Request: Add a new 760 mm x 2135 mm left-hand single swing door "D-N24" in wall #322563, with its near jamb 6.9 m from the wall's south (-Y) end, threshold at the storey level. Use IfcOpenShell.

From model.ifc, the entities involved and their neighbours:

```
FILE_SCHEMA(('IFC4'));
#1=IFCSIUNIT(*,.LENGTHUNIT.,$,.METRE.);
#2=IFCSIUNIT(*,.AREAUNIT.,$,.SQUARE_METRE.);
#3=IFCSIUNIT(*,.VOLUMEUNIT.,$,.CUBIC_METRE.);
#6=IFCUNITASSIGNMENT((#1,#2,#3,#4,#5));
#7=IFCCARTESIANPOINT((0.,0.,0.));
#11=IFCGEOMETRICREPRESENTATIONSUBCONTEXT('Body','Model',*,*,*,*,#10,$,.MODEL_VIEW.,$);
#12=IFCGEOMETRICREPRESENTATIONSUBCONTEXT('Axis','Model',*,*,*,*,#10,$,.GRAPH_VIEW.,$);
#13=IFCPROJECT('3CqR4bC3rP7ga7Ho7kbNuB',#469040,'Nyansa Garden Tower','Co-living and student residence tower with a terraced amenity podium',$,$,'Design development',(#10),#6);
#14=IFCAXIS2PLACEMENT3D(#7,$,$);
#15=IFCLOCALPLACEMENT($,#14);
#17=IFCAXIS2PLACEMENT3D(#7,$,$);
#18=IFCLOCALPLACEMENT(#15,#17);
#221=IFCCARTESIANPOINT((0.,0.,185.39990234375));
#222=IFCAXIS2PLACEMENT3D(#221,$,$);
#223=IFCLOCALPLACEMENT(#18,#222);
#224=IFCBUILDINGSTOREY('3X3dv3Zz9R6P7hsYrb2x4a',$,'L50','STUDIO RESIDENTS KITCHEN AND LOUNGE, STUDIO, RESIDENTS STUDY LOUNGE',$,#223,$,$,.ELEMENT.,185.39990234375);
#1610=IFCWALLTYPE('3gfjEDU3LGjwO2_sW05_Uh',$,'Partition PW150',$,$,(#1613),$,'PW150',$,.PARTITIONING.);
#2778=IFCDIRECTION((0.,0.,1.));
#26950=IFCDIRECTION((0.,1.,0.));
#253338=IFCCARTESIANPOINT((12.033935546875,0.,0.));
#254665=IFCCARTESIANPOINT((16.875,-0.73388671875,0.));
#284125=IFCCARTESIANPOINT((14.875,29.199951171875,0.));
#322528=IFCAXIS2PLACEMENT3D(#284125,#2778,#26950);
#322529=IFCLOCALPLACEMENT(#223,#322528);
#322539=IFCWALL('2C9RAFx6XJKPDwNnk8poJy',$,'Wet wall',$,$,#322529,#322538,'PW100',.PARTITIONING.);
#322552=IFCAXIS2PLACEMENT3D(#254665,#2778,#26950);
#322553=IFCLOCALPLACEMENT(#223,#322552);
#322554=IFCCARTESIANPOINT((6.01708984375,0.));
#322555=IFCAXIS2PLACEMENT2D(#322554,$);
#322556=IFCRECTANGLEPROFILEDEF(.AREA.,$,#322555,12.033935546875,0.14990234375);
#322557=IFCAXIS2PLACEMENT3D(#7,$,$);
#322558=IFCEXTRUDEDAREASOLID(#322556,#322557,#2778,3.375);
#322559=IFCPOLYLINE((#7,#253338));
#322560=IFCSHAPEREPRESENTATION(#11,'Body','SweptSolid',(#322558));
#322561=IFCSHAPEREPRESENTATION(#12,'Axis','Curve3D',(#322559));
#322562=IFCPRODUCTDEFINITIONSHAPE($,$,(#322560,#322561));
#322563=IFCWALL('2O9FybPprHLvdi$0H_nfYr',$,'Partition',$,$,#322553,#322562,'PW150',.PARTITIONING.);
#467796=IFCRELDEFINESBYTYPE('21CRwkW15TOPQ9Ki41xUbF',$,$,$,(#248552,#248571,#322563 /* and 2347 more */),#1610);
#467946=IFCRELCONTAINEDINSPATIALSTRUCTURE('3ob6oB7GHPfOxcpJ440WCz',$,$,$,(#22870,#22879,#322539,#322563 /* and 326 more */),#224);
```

```python
import numpy as np
import ifcopenshell
import ifcopenshell.api.feature
import ifcopenshell.api.geometry
import ifcopenshell.api.root
import ifcopenshell.api.spatial
import ifcopenshell.geom
import ifcopenshell.util.element
import ifcopenshell.util.placement
import ifcopenshell.util.representation
import ifcopenshell.util.shape
import ifcopenshell.util.unit

model = ifcopenshell.open("model.ifc")
unit_scale = ifcopenshell.util.unit.calculate_unit_scale(model)
settings = ifcopenshell.geom.settings()


def volume(element):
    """Net volume in cubic metres, openings subtracted."""
    shape = ifcopenshell.geom.create_shape(settings, element)
    return ifcopenshell.util.shape.get_volume(shape.geometry)


wall = model.by_id(322563)
storey = ifcopenshell.util.element.get_container(wall, ifc_class="IfcBuildingStorey")
context = ifcopenshell.util.representation.get_context(model, "Model", "Body", "MODEL_VIEW")
before = volume(wall)

width, height, from_end, sill = 0.76, 2.135, 6.9, 0.0  # metres

# The wall runs along its own X axis, and the end named is its -X end.
wall_shape = ifcopenshell.geom.create_shape(settings, wall)
x, y, z = ifcopenshell.util.shape.get_vertices(wall_shape.geometry).T
start = x.min() + from_end
face, thickness = float(y.min()), float(y.max() - y.min())
wall_matrix = ifcopenshell.util.placement.get_local_placement(wall.ObjectPlacement)
level = ifcopenshell.util.placement.get_local_placement(storey.ObjectPlacement)[2, 3]


def in_wall(x, y):
    """Placement at x, y metres in the wall's axes, at sill height."""
    matrix = wall_matrix.copy()
    matrix[:, 3] = wall_matrix @ np.array([x / unit_scale, y / unit_scale, 0.0, 1.0])
    matrix[2, 3] = level + sill / unit_scale
    return matrix


# Opening: a box that overshoots both wall faces by 50 mm.
opening = ifcopenshell.api.root.create_entity(model, ifc_class="IfcOpeningElement", predefined_type="OPENING")
box = ifcopenshell.api.geometry.add_wall_representation(
    model, context=context, length=width, height=height, thickness=thickness + 0.1
)
ifcopenshell.api.geometry.assign_representation(model, product=opening, representation=box)
ifcopenshell.api.geometry.edit_object_placement(model, product=opening, matrix=in_wall(start, face - 0.05), is_si=False)
ifcopenshell.api.feature.add_feature(model, feature=opening, element=wall)

door = ifcopenshell.api.root.create_entity(model, ifc_class="IfcDoor", name="D-N24", predefined_type="DOOR")
door.OverallWidth, door.OverallHeight = width / unit_scale, height / unit_scale
door.OperationType = "SINGLE_SWING_LEFT"
body = ifcopenshell.api.geometry.add_door_representation(
    model,
    context=context,
    overall_width=door.OverallWidth,
    overall_height=door.OverallHeight,
    operation_type="SINGLE_SWING_LEFT",
    lining_properties={"LiningDepth": thickness / unit_scale, "ThresholdDepth": thickness / unit_scale},
)
ifcopenshell.api.geometry.assign_representation(model, product=door, representation=body)
ifcopenshell.api.spatial.assign_container(model, products=[door], relating_structure=storey)
ifcopenshell.api.feature.add_filling(model, opening=opening, element=door)

# The lining spans the wall, so the door starts at the wall face.
ifcopenshell.api.geometry.edit_object_placement(model, product=door, matrix=in_wall(start, face), is_si=False)

after = volume(wall)

print(f"wall volume {before:.3f} -> {after:.3f} m3")

model.write("model-out.ifc")
```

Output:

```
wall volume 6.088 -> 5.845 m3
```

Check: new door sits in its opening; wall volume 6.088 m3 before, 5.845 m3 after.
